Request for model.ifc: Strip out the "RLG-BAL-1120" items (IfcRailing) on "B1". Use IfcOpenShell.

First a look at what the model holds.

```python
import ifcopenshell
import ifcopenshell.util.element

model = ifcopenshell.open("model.ifc")
print(model.schema)
storey = next(s for s in model.by_type("IfcBuildingStorey") if s.Name == "B1")
railings = [e for e in ifcopenshell.util.element.get_decomposition(storey) if e.is_a("IfcRailing")]
seen = {}
for e in railings:
    element_type = ifcopenshell.util.element.get_type(e)
    name = element_type.Name if element_type not in (None, e) else None
    seen[name] = seen.get(name, 0) + 1
for name, count in sorted(seen.items(), key=str):
    print(count, "x", name)
```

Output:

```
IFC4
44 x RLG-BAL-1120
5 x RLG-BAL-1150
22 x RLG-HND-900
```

```python
import ifcopenshell
import ifcopenshell.api.root
import ifcopenshell.util.element

model = ifcopenshell.open("model.ifc")

storey = next(s for s in model.by_type("IfcBuildingStorey") if s.Name == "B1")
railings = [e for e in ifcopenshell.util.element.get_decomposition(storey) if e.is_a("IfcRailing")]
targets = [e for e in railings if (t := ifcopenshell.util.element.get_type(e)) not in (None, e) and t.Name == "RLG-BAL-1120"]

for e in targets:
    ifcopenshell.api.root.remove_product(model, product=e)
print(len(targets), "removed")

model.write("model_rev.ifc")
```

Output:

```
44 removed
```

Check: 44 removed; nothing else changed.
